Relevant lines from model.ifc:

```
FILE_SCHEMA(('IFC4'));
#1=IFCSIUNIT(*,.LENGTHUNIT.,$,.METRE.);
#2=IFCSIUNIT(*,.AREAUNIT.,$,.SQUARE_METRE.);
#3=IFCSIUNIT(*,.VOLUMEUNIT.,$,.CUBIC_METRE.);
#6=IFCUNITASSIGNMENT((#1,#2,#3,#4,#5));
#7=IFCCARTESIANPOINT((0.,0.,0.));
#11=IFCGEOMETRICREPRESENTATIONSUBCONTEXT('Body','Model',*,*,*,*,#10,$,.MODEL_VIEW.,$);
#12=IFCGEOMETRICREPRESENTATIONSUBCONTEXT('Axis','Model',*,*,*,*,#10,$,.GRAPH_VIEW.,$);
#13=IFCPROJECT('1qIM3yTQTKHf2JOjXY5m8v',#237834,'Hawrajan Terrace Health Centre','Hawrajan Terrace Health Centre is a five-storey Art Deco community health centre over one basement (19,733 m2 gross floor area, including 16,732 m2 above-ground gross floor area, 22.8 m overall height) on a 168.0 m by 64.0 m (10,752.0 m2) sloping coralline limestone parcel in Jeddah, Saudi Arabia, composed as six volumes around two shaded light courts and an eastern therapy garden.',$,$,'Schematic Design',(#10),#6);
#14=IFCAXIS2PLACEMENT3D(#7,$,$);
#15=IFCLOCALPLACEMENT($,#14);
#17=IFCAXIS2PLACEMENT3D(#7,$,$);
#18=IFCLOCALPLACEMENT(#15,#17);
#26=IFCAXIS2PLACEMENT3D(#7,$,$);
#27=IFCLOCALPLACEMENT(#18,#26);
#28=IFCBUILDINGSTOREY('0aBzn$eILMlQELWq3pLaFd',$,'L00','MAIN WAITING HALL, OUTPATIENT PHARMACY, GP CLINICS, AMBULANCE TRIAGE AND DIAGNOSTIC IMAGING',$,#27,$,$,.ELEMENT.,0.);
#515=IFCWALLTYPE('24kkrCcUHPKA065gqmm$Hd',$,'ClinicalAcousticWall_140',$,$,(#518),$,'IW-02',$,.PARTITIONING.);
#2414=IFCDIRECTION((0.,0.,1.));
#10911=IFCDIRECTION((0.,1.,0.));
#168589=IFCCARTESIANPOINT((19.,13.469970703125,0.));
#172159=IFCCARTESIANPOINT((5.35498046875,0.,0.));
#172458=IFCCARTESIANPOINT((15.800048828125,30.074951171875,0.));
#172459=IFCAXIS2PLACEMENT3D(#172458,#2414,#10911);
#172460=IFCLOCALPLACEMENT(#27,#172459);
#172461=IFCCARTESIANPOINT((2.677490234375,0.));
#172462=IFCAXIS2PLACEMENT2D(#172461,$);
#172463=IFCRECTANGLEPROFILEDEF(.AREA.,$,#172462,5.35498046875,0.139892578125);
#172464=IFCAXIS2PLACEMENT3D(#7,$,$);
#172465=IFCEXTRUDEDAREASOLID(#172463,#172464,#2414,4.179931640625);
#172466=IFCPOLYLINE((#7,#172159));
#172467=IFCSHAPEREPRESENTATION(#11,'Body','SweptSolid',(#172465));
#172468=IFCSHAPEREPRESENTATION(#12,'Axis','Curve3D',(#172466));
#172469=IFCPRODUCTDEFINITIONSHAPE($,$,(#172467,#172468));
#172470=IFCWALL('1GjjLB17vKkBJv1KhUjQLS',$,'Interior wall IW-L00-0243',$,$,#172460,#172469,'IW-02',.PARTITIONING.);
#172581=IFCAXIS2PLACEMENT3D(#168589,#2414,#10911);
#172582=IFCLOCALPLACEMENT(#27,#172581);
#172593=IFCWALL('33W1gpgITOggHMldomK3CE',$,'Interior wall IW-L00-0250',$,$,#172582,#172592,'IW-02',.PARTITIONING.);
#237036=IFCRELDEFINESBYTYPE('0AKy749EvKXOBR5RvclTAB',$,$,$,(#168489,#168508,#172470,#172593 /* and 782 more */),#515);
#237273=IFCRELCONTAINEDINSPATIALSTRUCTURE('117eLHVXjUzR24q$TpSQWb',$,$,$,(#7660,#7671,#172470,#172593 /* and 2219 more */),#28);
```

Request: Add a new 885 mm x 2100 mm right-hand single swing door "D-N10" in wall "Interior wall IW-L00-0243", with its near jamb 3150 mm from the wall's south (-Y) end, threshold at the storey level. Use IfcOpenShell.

```python
import numpy as np
import ifcopenshell
import ifcopenshell.api.feature
import ifcopenshell.api.geometry
import ifcopenshell.api.root
import ifcopenshell.api.spatial
import ifcopenshell.geom
import ifcopenshell.util.element
import ifcopenshell.util.placement
import ifcopenshell.util.representation
import ifcopenshell.util.shape
import ifcopenshell.util.unit

model = ifcopenshell.open("model.ifc")
unit_scale = ifcopenshell.util.unit.calculate_unit_scale(model)
settings = ifcopenshell.geom.settings()


def volume(element):
    """Net volume in cubic metres, openings subtracted."""
    shape = ifcopenshell.geom.create_shape(settings, element)
    return ifcopenshell.util.shape.get_volume(shape.geometry)


wall = model.by_guid("1GjjLB17vKkBJv1KhUjQLS")
storey = ifcopenshell.util.element.get_container(wall, ifc_class="IfcBuildingStorey")
context = ifcopenshell.util.representation.get_context(model, "Model", "Body", "MODEL_VIEW")
before = volume(wall)

width, height, from_end, sill = 0.885, 2.1, 3.15, 0.0  # metres

# The wall runs along its own X axis, and the end named is its -X end.
wall_shape = ifcopenshell.geom.create_shape(settings, wall)
x, y, z = ifcopenshell.util.shape.get_vertices(wall_shape.geometry).T
start = x.min() + from_end
face, thickness = float(y.min()), float(y.max() - y.min())
wall_matrix = ifcopenshell.util.placement.get_local_placement(wall.ObjectPlacement)
level = ifcopenshell.util.placement.get_local_placement(storey.ObjectPlacement)[2, 3]


def in_wall(x, y):
    """Placement at x, y metres in the wall's axes, at sill height."""
    matrix = wall_matrix.copy()
    matrix[:, 3] = wall_matrix @ np.array([x / unit_scale, y / unit_scale, 0.0, 1.0])
    matrix[2, 3] = level + sill / unit_scale
    return matrix


# Opening: a box that overshoots both wall faces by 50 mm.
opening = ifcopenshell.api.root.create_entity(model, ifc_class="IfcOpeningElement", predefined_type="OPENING")
box = ifcopenshell.api.geometry.add_wall_representation(
    model, context=context, length=width, height=height, thickness=thickness + 0.1
)
ifcopenshell.api.geometry.assign_representation(model, product=opening, representation=box)
ifcopenshell.api.geometry.edit_object_placement(model, product=opening, matrix=in_wall(start, face - 0.05), is_si=False)
ifcopenshell.api.feature.add_feature(model, feature=opening, element=wall)

door = ifcopenshell.api.root.create_entity(model, ifc_class="IfcDoor", name="D-N10", predefined_type="DOOR")
door.OverallWidth, door.OverallHeight = width / unit_scale, height / unit_scale
door.OperationType = "SINGLE_SWING_RIGHT"
body = ifcopenshell.api.geometry.add_door_representation(
    model,
    context=context,
    overall_width=door.OverallWidth,
    overall_height=door.OverallHeight,
    operation_type="SINGLE_SWING_RIGHT",
    lining_properties={"LiningDepth": thickness / unit_scale, "ThresholdDepth": thickness / unit_scale},
)
ifcopenshell.api.geometry.assign_representation(model, product=door, representation=body)
ifcopenshell.api.spatial.assign_container(model, products=[door], relating_structure=storey)
ifcopenshell.api.feature.add_filling(model, opening=opening, element=door)

# The lining spans the wall, so the door starts at the wall face.
ifcopenshell.api.geometry.edit_object_placement(model, product=door, matrix=in_wall(start, face), is_si=False)

after = volume(wall)

print(f"wall volume {before:.3f} -> {after:.3f} m3")

model.write("model_edited.ifc")
```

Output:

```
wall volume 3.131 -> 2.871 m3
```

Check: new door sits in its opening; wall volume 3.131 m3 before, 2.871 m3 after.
